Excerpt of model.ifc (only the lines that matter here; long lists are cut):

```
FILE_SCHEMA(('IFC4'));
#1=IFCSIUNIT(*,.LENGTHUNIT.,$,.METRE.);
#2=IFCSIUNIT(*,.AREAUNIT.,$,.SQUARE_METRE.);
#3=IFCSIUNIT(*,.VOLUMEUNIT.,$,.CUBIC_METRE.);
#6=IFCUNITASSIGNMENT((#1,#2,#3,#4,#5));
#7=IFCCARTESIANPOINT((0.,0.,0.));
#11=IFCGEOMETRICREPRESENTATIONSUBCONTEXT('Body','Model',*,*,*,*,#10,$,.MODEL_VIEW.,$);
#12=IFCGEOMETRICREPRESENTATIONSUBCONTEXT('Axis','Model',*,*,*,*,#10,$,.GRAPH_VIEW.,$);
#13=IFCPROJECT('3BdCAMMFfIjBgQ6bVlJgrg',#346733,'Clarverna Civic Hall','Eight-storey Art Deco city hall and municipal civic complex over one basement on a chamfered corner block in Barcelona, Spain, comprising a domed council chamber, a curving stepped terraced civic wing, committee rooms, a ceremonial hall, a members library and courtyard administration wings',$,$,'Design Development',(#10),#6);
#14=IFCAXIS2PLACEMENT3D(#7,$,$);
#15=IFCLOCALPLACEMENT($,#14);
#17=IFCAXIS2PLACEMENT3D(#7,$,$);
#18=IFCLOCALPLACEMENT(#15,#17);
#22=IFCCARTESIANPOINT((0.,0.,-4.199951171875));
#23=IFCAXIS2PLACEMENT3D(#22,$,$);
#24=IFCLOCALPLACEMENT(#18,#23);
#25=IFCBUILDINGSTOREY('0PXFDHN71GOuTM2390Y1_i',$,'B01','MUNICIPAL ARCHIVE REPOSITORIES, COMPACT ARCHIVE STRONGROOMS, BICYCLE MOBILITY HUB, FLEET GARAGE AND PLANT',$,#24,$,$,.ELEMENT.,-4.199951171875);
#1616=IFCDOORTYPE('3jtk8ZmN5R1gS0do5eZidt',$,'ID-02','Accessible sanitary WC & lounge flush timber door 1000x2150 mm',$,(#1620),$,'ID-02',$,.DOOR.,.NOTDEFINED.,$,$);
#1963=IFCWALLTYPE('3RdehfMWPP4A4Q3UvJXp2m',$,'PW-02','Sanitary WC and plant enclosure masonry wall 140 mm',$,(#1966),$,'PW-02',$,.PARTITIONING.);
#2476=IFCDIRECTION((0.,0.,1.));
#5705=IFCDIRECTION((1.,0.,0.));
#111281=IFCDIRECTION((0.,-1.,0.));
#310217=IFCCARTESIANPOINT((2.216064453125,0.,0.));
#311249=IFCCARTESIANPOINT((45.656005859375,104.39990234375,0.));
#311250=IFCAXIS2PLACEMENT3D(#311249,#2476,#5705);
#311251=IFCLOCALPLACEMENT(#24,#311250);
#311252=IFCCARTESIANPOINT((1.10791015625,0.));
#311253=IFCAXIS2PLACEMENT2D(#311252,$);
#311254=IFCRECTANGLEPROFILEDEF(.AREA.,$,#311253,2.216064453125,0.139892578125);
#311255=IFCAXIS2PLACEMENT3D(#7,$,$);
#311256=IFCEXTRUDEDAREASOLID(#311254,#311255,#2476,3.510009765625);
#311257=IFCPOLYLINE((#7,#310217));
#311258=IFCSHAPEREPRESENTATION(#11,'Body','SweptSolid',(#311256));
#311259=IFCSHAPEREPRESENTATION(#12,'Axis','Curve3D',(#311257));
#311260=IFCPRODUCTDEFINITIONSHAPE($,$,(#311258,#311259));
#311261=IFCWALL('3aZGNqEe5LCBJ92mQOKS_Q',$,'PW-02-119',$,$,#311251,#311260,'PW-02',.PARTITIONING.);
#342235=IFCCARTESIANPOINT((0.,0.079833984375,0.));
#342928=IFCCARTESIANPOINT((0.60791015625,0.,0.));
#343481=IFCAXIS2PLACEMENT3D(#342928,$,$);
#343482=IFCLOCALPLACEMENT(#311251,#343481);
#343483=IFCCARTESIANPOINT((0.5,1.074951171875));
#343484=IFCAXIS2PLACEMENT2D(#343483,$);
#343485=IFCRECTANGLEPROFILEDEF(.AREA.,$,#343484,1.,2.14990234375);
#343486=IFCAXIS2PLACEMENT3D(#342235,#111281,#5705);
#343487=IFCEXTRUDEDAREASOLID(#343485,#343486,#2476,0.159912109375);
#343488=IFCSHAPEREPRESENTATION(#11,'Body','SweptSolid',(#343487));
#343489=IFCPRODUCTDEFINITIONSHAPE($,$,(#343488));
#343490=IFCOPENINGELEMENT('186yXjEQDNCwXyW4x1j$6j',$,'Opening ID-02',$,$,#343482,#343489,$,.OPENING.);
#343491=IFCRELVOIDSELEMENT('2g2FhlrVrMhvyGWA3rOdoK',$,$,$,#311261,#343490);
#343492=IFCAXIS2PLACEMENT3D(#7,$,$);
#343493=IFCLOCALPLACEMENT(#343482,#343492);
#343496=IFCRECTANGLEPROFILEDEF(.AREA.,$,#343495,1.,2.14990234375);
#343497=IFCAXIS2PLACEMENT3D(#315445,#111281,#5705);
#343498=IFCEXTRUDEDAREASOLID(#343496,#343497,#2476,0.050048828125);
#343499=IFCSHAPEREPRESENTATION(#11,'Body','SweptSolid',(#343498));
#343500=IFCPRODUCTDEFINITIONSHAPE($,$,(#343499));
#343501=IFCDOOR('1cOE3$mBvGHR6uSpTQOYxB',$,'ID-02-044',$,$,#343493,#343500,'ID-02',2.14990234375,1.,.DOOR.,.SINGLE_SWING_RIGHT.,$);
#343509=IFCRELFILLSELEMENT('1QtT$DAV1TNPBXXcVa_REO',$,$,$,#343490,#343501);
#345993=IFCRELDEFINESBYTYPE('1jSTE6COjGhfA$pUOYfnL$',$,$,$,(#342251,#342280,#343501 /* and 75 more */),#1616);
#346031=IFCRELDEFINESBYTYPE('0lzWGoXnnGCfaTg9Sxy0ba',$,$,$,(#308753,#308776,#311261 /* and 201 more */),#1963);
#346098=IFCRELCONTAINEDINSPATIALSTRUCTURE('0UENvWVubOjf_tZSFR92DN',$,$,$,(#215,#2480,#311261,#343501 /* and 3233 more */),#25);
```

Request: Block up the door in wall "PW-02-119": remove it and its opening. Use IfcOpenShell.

```python
import ifcopenshell
import ifcopenshell.api.feature
import ifcopenshell.api.root
import ifcopenshell.geom
import ifcopenshell.util.shape

model = ifcopenshell.open("model.ifc")
settings = ifcopenshell.geom.settings()


def volume(element):
    """Net volume in cubic metres, openings subtracted."""
    shape = ifcopenshell.geom.create_shape(settings, element)
    return ifcopenshell.util.shape.get_volume(shape.geometry)


door = model.by_id(343501)
opening = door.FillsVoids[0].RelatingOpeningElement
wall = opening.VoidsElements[0].RelatingBuildingElement
before = volume(wall)

ifcopenshell.api.root.remove_product(model, product=door)
ifcopenshell.api.feature.remove_feature(model, feature=opening)

after = volume(wall)

print(f"wall volume {before:.3f} -> {after:.3f} m3")

model.write("model_v2.ifc")
```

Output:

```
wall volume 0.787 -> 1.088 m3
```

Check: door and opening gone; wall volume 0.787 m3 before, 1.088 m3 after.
